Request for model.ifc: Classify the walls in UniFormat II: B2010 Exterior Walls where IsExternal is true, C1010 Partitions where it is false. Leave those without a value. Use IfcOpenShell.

First a look at what the model holds.

```python
import ifcopenshell
import ifcopenshell.util.element

model = ifcopenshell.open("model.ifc")
print(model.schema)
print("classifications:", [c.Name for c in model.by_type("IfcClassification")])
values = [ifcopenshell.util.element.get_pset(e, "Pset_WallCommon", "IsExternal") for e in model.by_type("IfcWall")]
for value in (True, False, None):
    print("IsExternal", value, values.count(value))
```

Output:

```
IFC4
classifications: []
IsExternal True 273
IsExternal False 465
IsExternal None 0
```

```python
import ifcopenshell
import ifcopenshell.api.classification
import ifcopenshell.util.element

model = ifcopenshell.open("model.ifc")

system = ifcopenshell.api.classification.add_classification(model, classification="UniFormat II")

walls = model.by_type("IfcWall")
external = {e: ifcopenshell.util.element.get_pset(e, "Pset_WallCommon", "IsExternal") for e in walls}
for flag, code, name in ((True, "B2010", "Exterior Walls"), (False, "C1010", "Partitions")):
    products = [e for e in walls if external[e] is flag]
    ifcopenshell.api.classification.add_reference(
        model, products=products, classification=system, identification=code, name=name
    )
    print(code, len(products))

model.write("model_updated.ifc")
```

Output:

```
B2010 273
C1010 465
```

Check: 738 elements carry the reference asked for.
